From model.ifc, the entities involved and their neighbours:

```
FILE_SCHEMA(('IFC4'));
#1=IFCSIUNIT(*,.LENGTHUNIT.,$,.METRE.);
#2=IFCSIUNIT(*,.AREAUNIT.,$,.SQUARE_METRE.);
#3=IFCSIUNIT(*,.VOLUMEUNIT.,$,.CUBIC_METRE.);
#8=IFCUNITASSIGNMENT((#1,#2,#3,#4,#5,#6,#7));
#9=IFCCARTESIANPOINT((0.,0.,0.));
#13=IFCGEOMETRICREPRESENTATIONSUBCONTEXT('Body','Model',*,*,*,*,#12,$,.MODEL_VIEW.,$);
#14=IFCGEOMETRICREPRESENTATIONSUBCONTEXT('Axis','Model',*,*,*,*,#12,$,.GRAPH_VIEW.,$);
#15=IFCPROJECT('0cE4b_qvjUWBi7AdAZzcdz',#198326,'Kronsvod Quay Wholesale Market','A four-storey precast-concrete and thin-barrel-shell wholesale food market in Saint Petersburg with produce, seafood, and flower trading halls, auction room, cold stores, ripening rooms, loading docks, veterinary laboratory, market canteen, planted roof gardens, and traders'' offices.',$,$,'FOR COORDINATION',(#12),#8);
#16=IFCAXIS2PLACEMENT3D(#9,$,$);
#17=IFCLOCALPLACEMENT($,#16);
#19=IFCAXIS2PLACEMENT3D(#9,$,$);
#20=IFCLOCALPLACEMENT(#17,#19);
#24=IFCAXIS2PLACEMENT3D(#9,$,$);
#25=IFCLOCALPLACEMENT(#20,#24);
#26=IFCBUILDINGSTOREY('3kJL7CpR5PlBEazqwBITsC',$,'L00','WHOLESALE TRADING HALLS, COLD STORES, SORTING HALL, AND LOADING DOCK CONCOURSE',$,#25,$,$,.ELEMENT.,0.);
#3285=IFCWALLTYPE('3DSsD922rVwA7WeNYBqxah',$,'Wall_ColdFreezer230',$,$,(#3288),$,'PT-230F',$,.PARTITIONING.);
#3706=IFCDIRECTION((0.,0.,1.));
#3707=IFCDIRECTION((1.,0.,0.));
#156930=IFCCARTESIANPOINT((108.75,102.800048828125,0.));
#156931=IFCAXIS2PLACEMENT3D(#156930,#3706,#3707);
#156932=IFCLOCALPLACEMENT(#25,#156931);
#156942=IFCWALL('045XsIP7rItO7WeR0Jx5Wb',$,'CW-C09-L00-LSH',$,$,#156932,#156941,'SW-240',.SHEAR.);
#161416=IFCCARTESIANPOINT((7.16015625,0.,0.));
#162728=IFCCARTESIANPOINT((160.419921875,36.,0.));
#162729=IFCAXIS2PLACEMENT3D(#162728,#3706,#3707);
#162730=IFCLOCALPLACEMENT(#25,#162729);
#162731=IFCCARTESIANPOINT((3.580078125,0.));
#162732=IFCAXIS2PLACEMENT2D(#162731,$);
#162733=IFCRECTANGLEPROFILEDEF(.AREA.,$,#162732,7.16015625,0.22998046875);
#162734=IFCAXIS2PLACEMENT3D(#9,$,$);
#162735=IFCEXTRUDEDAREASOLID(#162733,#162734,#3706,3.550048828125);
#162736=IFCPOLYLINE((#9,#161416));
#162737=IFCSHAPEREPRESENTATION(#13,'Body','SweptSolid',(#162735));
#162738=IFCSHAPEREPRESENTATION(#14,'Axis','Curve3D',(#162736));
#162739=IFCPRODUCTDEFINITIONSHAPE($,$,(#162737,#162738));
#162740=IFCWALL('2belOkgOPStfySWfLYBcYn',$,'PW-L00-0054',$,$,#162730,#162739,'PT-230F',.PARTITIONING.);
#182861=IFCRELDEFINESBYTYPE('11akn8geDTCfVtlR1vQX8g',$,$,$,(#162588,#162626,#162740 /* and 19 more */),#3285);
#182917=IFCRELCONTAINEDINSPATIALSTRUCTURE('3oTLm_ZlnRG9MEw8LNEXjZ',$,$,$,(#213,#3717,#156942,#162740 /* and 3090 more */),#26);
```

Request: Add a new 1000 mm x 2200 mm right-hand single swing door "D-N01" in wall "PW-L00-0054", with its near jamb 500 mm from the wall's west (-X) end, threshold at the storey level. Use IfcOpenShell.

```python
import numpy as np
import ifcopenshell
import ifcopenshell.api.feature
import ifcopenshell.api.geometry
import ifcopenshell.api.root
import ifcopenshell.api.spatial
import ifcopenshell.geom
import ifcopenshell.util.element
import ifcopenshell.util.placement
import ifcopenshell.util.representation
import ifcopenshell.util.shape
import ifcopenshell.util.unit

model = ifcopenshell.open("model.ifc")
unit_scale = ifcopenshell.util.unit.calculate_unit_scale(model)
settings = ifcopenshell.geom.settings()


def volume(element):
    """Net volume in cubic metres, openings subtracted."""
    shape = ifcopenshell.geom.create_shape(settings, element)
    return ifcopenshell.util.shape.get_volume(shape.geometry)


wall = model.by_guid("2belOkgOPStfySWfLYBcYn")
storey = ifcopenshell.util.element.get_container(wall, ifc_class="IfcBuildingStorey")
context = ifcopenshell.util.representation.get_context(model, "Model", "Body", "MODEL_VIEW")
before = volume(wall)

width, height, from_end, sill = 1, 2.2, 0.5, 0.0  # metres

# The wall runs along its own X axis, and the end named is its -X end.
wall_shape = ifcopenshell.geom.create_shape(settings, wall)
x, y, z = ifcopenshell.util.shape.get_vertices(wall_shape.geometry).T
start = x.min() + from_end
face, thickness = float(y.min()), float(y.max() - y.min())
wall_matrix = ifcopenshell.util.placement.get_local_placement(wall.ObjectPlacement)
level = ifcopenshell.util.placement.get_local_placement(storey.ObjectPlacement)[2, 3]


def in_wall(x, y):
    """Placement at x, y metres in the wall's axes, at sill height."""
    matrix = wall_matrix.copy()
    matrix[:, 3] = wall_matrix @ np.array([x / unit_scale, y / unit_scale, 0.0, 1.0])
    matrix[2, 3] = level + sill / unit_scale
    return matrix


# Opening: a box that overshoots both wall faces by 50 mm.
opening = ifcopenshell.api.root.create_entity(model, ifc_class="IfcOpeningElement", predefined_type="OPENING")
box = ifcopenshell.api.geometry.add_wall_representation(
    model, context=context, length=width, height=height, thickness=thickness + 0.1
)
ifcopenshell.api.geometry.assign_representation(model, product=opening, representation=box)
ifcopenshell.api.geometry.edit_object_placement(model, product=opening, matrix=in_wall(start, face - 0.05), is_si=False)
ifcopenshell.api.feature.add_feature(model, feature=opening, element=wall)

door = ifcopenshell.api.root.create_entity(model, ifc_class="IfcDoor", name="D-N01", predefined_type="DOOR")
door.OverallWidth, door.OverallHeight = width / unit_scale, height / unit_scale
door.OperationType = "SINGLE_SWING_RIGHT"
body = ifcopenshell.api.geometry.add_door_representation(
    model,
    context=context,
    overall_width=door.OverallWidth,
    overall_height=door.OverallHeight,
    operation_type="SINGLE_SWING_RIGHT",
    lining_properties={"LiningDepth": thickness / unit_scale, "ThresholdDepth": thickness / unit_scale},
)
ifcopenshell.api.geometry.assign_representation(model, product=door, representation=body)
ifcopenshell.api.spatial.assign_container(model, products=[door], relating_structure=storey)
ifcopenshell.api.feature.add_filling(model, opening=opening, element=door)

# The lining spans the wall, so the door starts at the wall face.
ifcopenshell.api.geometry.edit_object_placement(model, product=door, matrix=in_wall(start, face), is_si=False)

after = volume(wall)

print(f"wall volume {before:.3f} -> {after:.3f} m3")

model.write("model_edited.ifc")
```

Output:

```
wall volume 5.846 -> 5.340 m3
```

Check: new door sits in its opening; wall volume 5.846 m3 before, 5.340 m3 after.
